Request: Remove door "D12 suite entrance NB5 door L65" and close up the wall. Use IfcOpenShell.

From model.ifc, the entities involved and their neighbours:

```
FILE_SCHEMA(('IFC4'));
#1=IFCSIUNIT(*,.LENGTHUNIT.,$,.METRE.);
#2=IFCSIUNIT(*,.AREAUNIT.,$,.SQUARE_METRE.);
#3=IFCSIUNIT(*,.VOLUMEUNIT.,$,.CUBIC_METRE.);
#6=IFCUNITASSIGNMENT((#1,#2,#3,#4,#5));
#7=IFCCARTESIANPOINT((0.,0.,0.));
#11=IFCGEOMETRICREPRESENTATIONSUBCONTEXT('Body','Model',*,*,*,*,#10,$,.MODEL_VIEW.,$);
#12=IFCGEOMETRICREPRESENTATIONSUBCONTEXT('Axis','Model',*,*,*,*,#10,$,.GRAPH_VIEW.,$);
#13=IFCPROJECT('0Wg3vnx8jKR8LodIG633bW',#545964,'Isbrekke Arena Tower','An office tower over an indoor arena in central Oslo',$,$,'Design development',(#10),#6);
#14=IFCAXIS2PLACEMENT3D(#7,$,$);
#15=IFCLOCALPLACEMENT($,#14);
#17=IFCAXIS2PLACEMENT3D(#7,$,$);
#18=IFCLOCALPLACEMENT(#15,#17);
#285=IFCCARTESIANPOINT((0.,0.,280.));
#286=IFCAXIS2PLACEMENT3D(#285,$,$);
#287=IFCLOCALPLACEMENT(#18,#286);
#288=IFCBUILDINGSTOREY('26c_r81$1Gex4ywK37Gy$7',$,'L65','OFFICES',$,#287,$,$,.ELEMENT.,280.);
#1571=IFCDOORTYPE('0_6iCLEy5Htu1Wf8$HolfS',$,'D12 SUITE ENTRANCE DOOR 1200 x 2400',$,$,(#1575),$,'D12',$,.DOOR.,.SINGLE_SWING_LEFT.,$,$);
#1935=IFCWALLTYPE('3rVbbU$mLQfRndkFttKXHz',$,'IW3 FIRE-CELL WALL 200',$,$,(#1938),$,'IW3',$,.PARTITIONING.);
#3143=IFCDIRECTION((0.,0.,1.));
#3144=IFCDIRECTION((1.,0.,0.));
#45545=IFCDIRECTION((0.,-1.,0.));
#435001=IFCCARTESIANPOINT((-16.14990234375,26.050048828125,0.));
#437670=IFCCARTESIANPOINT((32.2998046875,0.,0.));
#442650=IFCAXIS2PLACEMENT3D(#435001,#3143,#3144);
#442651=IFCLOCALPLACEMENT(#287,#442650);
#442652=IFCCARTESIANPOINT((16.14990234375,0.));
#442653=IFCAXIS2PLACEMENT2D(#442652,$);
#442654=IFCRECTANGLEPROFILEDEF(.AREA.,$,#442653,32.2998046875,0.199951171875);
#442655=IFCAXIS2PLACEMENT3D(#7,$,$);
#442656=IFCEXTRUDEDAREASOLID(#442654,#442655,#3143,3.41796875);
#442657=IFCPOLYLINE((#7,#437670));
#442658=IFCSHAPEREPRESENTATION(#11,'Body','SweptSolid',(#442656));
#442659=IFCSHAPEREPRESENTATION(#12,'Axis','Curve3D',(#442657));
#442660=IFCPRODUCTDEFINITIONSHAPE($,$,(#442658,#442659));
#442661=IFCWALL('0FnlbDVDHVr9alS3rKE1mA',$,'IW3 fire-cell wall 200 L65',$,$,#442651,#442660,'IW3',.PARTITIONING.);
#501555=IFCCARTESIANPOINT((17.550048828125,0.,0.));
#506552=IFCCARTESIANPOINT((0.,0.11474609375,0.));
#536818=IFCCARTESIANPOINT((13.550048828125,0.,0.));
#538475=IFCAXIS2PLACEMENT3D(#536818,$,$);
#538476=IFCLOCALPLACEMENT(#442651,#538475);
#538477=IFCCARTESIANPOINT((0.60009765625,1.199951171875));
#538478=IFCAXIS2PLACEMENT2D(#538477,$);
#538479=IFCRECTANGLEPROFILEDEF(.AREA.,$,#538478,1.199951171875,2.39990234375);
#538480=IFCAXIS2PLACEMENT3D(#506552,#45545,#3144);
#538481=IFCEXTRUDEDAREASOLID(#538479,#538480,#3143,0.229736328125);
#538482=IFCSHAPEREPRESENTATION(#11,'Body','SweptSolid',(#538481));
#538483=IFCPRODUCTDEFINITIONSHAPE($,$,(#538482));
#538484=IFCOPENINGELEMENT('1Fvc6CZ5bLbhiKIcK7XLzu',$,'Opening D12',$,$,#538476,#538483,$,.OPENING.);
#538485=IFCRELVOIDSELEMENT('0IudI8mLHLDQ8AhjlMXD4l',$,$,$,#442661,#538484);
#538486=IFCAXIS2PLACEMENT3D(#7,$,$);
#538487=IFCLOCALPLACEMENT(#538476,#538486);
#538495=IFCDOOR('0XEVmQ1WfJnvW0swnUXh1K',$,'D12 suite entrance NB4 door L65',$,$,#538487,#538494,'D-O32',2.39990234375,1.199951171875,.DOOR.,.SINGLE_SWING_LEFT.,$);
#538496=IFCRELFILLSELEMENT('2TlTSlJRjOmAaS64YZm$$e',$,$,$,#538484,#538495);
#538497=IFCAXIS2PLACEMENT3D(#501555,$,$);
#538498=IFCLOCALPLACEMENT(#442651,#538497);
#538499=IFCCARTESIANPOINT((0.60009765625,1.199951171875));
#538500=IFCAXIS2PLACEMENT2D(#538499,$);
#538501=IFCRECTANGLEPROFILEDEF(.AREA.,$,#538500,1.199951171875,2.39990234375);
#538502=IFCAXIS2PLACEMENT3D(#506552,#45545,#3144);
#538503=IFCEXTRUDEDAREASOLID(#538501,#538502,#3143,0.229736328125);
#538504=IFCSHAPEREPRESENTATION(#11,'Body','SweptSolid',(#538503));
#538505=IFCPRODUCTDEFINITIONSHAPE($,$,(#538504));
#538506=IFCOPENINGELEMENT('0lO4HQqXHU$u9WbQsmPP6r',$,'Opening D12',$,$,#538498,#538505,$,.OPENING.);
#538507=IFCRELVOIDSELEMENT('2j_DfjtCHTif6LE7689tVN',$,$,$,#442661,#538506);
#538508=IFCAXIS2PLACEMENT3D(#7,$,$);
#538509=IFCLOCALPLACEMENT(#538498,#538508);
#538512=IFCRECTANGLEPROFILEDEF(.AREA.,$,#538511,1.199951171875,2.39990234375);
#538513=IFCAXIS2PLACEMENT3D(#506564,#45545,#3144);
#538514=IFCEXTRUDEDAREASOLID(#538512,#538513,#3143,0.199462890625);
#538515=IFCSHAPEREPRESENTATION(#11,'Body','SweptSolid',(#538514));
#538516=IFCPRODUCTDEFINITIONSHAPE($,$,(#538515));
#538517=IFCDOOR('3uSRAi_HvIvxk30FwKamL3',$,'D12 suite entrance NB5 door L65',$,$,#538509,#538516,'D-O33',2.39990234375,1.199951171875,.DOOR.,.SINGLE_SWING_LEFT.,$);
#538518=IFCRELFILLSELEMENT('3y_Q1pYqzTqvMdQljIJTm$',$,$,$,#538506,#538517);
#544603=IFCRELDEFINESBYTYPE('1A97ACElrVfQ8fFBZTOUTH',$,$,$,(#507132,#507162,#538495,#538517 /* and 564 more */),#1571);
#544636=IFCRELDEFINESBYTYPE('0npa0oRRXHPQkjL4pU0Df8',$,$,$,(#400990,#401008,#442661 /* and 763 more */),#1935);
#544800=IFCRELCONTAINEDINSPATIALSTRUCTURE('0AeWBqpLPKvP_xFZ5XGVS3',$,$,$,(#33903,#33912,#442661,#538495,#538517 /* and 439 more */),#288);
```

```python
import ifcopenshell
import ifcopenshell.api.feature
import ifcopenshell.api.root
import ifcopenshell.geom
import ifcopenshell.util.shape

model = ifcopenshell.open("model.ifc")
settings = ifcopenshell.geom.settings()


def volume(element):
    """Net volume in cubic metres, openings subtracted."""
    shape = ifcopenshell.geom.create_shape(settings, element)
    return ifcopenshell.util.shape.get_volume(shape.geometry)


door = model.by_id(538517)
opening = door.FillsVoids[0].RelatingOpeningElement
wall = opening.VoidsElements[0].RelatingBuildingElement
before = volume(wall)

ifcopenshell.api.root.remove_product(model, product=door)
ifcopenshell.api.feature.remove_feature(model, feature=opening)

after = volume(wall)

print(f"wall volume {before:.3f} -> {after:.3f} m3")

model.write("model_edited.ifc")
```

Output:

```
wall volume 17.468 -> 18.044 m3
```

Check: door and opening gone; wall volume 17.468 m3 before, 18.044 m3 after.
